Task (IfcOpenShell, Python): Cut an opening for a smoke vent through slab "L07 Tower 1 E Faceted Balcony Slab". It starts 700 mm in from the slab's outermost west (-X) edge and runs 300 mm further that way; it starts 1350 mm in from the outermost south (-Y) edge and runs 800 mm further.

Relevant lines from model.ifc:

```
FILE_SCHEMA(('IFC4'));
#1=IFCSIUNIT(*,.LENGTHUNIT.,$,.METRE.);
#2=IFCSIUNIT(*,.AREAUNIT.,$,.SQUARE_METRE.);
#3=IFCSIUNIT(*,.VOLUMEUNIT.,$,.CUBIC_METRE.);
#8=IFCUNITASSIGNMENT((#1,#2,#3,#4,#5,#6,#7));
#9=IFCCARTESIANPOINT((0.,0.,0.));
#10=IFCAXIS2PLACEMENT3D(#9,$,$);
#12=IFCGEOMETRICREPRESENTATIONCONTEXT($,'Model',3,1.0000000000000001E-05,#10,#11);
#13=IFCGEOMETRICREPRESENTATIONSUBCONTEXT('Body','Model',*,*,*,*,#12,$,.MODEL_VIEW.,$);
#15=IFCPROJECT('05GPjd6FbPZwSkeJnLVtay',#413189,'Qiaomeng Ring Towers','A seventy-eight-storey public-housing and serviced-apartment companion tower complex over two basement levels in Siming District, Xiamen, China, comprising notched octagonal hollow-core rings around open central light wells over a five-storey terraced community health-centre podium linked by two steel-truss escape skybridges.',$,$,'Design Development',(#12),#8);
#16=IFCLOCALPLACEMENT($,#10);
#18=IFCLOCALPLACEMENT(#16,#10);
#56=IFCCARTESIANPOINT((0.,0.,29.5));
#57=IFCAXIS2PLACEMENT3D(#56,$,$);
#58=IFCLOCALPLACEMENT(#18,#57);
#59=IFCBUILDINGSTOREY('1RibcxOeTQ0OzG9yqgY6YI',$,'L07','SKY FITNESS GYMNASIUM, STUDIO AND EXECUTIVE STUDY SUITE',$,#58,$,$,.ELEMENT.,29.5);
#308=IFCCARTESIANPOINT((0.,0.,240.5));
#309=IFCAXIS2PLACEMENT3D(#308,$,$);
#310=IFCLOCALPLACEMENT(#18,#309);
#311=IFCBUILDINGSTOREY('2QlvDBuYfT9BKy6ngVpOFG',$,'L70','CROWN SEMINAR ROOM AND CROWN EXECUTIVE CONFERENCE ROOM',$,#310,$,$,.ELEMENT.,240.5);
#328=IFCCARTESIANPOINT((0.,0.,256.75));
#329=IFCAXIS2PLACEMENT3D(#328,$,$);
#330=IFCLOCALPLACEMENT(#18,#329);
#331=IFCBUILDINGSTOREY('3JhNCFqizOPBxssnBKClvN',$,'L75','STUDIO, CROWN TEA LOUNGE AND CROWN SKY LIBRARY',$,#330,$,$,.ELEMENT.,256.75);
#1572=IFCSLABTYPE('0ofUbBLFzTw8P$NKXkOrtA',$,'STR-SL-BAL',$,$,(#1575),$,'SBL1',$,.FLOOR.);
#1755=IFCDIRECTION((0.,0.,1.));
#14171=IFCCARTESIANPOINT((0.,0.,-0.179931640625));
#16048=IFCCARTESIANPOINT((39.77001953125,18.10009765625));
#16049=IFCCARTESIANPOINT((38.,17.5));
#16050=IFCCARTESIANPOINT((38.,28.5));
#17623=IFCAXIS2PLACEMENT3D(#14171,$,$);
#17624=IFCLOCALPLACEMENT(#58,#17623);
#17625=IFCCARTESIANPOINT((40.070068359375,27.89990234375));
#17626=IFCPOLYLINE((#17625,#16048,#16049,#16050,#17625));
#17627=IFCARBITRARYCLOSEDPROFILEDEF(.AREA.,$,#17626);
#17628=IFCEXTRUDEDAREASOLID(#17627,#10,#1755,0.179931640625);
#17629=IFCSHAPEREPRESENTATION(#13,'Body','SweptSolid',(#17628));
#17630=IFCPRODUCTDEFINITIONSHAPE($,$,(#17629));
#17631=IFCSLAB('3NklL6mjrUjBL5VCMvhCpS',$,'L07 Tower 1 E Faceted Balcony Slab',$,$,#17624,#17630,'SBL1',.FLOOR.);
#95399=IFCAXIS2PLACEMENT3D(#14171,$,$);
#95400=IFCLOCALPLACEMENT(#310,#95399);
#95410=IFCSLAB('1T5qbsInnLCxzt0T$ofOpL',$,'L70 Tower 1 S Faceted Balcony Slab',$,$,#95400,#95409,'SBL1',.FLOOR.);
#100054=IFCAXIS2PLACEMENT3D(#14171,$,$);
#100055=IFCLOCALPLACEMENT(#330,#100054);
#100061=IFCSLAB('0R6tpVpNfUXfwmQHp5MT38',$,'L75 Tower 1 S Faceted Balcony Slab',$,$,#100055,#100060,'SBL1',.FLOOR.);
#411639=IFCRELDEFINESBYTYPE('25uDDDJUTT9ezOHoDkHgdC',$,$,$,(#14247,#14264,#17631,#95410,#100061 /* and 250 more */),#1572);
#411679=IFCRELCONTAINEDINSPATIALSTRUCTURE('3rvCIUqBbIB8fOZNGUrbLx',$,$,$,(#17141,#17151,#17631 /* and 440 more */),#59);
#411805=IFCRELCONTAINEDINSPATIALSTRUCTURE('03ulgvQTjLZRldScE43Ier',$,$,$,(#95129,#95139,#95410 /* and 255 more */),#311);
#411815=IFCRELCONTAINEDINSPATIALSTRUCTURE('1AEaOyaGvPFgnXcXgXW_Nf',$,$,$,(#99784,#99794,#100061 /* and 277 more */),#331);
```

```python
import numpy as np
import ifcopenshell
import ifcopenshell.api.feature
import ifcopenshell.api.geometry
import ifcopenshell.api.root
import ifcopenshell.geom
import ifcopenshell.util.placement
import ifcopenshell.util.representation
import ifcopenshell.util.shape
import ifcopenshell.util.unit

model = ifcopenshell.open("model.ifc")
unit_scale = ifcopenshell.util.unit.calculate_unit_scale(model)
settings = ifcopenshell.geom.settings()


def volume(element):
    """Net volume in cubic metres, openings subtracted."""
    shape = ifcopenshell.geom.create_shape(settings, element)
    return ifcopenshell.util.shape.get_volume(shape.geometry)


slab = model.by_id(17631)
before = volume(slab)

# Extent in the slab's own axes, in metres. The edges named are its -X and -Y sides.
slab_shape = ifcopenshell.geom.create_shape(settings, slab)
vertices = ifcopenshell.util.shape.get_vertices(slab_shape.geometry)
x_min, y_min, bottom = vertices.min(axis=0)
top = vertices[:, 2].max()

opening = ifcopenshell.api.root.create_entity(model, ifc_class="IfcOpeningElement", name="Smoke vent opening", predefined_type="OPENING")
context = ifcopenshell.util.representation.get_context(model, "Model", "Body", "MODEL_VIEW")
width, depth = 0.3, 0.8
outline = [(0.0, 0.0), (width, 0.0), (width, depth), (0.0, depth), (0.0, 0.0)]
# Overshoot both faces by 50 mm so the cut is clean.
shape = ifcopenshell.api.geometry.add_slab_representation(
    model, context=context, depth=top - bottom + 0.1, polyline=outline
)
ifcopenshell.api.geometry.assign_representation(model, product=opening, representation=shape)

matrix = ifcopenshell.util.placement.get_local_placement(slab.ObjectPlacement)
matrix[:, 3] = matrix @ np.append(np.array([x_min + 0.7, y_min + 1.35, bottom - 0.05]) / unit_scale, 1.0)
ifcopenshell.api.geometry.edit_object_placement(model, product=opening, matrix=matrix, is_si=False)
ifcopenshell.api.feature.add_feature(model, feature=opening, element=slab)

after = volume(slab)

print(f"slab volume {before:.3f} -> {after:.3f} m3")

model.write("model_rev.ifc")
```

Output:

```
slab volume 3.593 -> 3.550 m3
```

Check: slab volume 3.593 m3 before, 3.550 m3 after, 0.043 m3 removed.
